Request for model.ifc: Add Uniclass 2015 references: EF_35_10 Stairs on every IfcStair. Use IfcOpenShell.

First a look at what the model holds.

```python
import ifcopenshell

model = ifcopenshell.open("model.ifc")
print(model.schema)
print("classifications:", [c.Name for c in model.by_type("IfcClassification")])
for ifc_class in ("IfcDoor", "IfcRoof", "IfcStair", "IfcWall", "IfcWindow"):
    print(ifc_class, len(model.by_type(ifc_class)))
```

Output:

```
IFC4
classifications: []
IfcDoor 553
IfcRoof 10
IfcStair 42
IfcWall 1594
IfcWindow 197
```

```python
import ifcopenshell
import ifcopenshell.api.classification

model = ifcopenshell.open("model.ifc")

system = ifcopenshell.api.classification.add_classification(model, classification="Uniclass 2015")

codes = {
    "IfcStair": ("EF_35_10", "Stairs"),
}
for ifc_class, (code, name) in codes.items():
    products = model.by_type(ifc_class)
    ifcopenshell.api.classification.add_reference(
        model, products=products, classification=system, identification=code, name=name
    )
    print(code, len(products))

model.write("model_rev.ifc")
```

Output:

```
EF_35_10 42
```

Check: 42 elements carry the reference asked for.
